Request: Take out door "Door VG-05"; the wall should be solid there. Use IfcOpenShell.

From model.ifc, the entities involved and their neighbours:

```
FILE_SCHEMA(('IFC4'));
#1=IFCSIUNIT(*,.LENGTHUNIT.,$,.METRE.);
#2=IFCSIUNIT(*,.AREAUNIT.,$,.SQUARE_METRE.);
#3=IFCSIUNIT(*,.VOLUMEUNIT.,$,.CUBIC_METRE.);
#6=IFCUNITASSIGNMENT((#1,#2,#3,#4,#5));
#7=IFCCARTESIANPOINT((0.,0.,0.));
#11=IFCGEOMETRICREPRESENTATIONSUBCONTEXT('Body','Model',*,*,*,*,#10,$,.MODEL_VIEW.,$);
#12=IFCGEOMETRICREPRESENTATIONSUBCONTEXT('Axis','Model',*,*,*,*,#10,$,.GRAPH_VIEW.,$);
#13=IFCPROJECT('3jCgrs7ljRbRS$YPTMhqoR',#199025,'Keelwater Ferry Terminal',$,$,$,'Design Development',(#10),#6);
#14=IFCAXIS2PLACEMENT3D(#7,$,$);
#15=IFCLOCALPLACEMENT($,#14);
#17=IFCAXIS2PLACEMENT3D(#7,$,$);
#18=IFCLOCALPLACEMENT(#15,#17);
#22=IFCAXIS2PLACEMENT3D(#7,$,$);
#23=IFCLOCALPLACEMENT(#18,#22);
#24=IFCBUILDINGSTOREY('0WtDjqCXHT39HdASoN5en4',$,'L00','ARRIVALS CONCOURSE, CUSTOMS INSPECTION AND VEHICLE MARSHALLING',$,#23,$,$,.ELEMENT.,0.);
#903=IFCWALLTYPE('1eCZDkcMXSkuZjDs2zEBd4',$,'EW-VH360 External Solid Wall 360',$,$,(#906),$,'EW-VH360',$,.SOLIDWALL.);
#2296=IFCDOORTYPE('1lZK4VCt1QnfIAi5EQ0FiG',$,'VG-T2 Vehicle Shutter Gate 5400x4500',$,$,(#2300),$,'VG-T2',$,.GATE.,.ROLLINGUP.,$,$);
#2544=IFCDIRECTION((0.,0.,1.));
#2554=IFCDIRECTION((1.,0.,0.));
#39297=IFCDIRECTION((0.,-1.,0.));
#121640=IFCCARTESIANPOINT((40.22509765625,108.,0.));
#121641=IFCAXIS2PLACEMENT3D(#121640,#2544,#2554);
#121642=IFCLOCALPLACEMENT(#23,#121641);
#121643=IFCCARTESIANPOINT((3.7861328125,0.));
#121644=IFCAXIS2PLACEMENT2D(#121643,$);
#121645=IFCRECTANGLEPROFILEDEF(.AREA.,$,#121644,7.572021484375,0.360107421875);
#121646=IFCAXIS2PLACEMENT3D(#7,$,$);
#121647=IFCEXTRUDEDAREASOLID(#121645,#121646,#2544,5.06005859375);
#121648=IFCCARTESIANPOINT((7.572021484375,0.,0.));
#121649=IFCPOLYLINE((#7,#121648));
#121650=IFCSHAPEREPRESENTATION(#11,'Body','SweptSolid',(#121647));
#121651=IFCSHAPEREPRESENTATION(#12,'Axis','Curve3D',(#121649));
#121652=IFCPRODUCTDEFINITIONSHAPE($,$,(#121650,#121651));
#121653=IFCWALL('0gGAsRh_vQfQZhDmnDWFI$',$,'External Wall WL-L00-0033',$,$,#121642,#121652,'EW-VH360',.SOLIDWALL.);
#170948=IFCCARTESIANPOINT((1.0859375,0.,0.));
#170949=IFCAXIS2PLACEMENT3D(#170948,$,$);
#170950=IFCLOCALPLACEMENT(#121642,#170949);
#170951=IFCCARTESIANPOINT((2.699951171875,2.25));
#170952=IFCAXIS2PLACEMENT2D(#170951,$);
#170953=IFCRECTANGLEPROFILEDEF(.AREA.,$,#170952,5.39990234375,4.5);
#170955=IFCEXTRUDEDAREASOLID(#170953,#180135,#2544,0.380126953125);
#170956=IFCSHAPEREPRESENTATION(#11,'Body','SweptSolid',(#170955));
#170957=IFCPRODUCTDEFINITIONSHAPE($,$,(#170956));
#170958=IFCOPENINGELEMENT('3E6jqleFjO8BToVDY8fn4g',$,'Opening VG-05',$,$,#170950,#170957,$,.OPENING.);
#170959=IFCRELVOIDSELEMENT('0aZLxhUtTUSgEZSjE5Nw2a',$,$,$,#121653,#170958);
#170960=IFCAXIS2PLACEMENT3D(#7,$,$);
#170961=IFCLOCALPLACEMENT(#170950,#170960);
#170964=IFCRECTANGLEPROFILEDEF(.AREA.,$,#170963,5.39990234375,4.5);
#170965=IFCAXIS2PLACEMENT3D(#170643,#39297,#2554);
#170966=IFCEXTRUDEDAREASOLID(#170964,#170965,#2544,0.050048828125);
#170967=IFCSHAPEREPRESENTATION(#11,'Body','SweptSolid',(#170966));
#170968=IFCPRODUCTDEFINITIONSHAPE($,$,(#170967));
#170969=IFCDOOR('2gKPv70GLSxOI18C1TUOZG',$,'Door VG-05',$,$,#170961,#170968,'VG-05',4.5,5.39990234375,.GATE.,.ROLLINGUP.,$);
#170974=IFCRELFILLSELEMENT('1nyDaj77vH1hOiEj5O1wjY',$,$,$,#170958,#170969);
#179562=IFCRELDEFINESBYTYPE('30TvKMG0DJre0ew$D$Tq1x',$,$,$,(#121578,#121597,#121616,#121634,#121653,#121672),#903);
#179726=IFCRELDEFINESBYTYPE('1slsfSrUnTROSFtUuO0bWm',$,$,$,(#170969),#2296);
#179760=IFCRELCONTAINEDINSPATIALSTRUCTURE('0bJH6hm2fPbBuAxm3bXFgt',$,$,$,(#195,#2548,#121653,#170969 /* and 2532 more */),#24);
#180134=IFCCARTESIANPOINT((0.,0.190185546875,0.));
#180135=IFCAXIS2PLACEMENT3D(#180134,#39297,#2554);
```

```python
import ifcopenshell
import ifcopenshell.api.feature
import ifcopenshell.api.root
import ifcopenshell.geom
import ifcopenshell.util.shape

model = ifcopenshell.open("model.ifc")
settings = ifcopenshell.geom.settings()


def volume(element):
    """Net volume in cubic metres, openings subtracted."""
    shape = ifcopenshell.geom.create_shape(settings, element)
    return ifcopenshell.util.shape.get_volume(shape.geometry)


door = model.by_guid("2gKPv70GLSxOI18C1TUOZG")
opening = door.FillsVoids[0].RelatingOpeningElement
wall = opening.VoidsElements[0].RelatingBuildingElement
before = volume(wall)

ifcopenshell.api.root.remove_product(model, product=door)
ifcopenshell.api.feature.remove_feature(model, feature=opening)

after = volume(wall)

print(f"wall volume {before:.3f} -> {after:.3f} m3")

model.write("model_v2.ifc")
```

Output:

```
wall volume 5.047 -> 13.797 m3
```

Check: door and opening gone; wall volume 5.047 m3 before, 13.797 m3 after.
